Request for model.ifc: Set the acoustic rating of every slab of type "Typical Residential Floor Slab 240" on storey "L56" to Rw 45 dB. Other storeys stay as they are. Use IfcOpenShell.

First a look at what the model holds.

```python
import ifcopenshell
import ifcopenshell.util.element

model = ifcopenshell.open("model.ifc")
print(model.schema)
storey = next(s for s in model.by_type("IfcBuildingStorey") if s.Name == "L56")
slabs = [e for e in ifcopenshell.util.element.get_decomposition(storey) if e.is_a("IfcSlab")]
seen = {}
for e in slabs:
    element_type = ifcopenshell.util.element.get_type(e)
    key = (element_type.Name if element_type != e and element_type else None, ifcopenshell.util.element.get_pset(e, "Pset_SlabCommon", "AcousticRating"))
    seen[key] = seen.get(key, 0) + 1
for (name, value), count in sorted(seen.items(), key=str):
    print(count, "x", name, "|", value)
```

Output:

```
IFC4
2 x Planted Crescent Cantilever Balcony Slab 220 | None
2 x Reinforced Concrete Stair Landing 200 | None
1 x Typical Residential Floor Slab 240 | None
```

```python
import ifcopenshell
import ifcopenshell.api.pset
import ifcopenshell.util.element

model = ifcopenshell.open("model.ifc")

storey = next(s for s in model.by_type("IfcBuildingStorey") if s.Name == "L56")
slabs = [e for e in ifcopenshell.util.element.get_decomposition(storey) if e.is_a("IfcSlab")]

count = 0
for e in slabs:
    element_type = ifcopenshell.util.element.get_type(e)
    if element_type in (None, e) or element_type.Name != "Typical Residential Floor Slab 240":
        continue
    # add_pset returns the element's existing set when there is one.
    pset = ifcopenshell.api.pset.add_pset(model, product=e, name="Pset_SlabCommon")
    ifcopenshell.api.pset.edit_pset(model, pset=pset, properties={"AcousticRating": "Rw 45 dB"})
    count += 1

print(count, "slabs updated")

model.write("model_edited.ifc")
```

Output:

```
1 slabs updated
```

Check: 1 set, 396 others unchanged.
